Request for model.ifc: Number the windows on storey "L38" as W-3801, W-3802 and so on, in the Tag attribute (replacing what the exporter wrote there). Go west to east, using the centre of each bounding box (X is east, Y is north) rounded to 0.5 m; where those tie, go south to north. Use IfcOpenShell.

First a look at what the model holds.

```python
import ifcopenshell
import ifcopenshell.util.element
import ifcopenshell.util.placement

model = ifcopenshell.open("model.ifc")
print(model.schema)
storey = next(s for s in model.by_type("IfcBuildingStorey") if s.Name == "L38")
windows = [e for e in ifcopenshell.util.element.get_decomposition(storey) if e.is_a("IfcWindow")]
for e in sorted(windows, key=lambda e: e.id()):
    origin = ifcopenshell.util.placement.get_local_placement(e.ObjectPlacement)[:3, 3]
    print(e.id(), e.Tag, e.Name, origin.round(2) + 0.0, sep=" | ")
```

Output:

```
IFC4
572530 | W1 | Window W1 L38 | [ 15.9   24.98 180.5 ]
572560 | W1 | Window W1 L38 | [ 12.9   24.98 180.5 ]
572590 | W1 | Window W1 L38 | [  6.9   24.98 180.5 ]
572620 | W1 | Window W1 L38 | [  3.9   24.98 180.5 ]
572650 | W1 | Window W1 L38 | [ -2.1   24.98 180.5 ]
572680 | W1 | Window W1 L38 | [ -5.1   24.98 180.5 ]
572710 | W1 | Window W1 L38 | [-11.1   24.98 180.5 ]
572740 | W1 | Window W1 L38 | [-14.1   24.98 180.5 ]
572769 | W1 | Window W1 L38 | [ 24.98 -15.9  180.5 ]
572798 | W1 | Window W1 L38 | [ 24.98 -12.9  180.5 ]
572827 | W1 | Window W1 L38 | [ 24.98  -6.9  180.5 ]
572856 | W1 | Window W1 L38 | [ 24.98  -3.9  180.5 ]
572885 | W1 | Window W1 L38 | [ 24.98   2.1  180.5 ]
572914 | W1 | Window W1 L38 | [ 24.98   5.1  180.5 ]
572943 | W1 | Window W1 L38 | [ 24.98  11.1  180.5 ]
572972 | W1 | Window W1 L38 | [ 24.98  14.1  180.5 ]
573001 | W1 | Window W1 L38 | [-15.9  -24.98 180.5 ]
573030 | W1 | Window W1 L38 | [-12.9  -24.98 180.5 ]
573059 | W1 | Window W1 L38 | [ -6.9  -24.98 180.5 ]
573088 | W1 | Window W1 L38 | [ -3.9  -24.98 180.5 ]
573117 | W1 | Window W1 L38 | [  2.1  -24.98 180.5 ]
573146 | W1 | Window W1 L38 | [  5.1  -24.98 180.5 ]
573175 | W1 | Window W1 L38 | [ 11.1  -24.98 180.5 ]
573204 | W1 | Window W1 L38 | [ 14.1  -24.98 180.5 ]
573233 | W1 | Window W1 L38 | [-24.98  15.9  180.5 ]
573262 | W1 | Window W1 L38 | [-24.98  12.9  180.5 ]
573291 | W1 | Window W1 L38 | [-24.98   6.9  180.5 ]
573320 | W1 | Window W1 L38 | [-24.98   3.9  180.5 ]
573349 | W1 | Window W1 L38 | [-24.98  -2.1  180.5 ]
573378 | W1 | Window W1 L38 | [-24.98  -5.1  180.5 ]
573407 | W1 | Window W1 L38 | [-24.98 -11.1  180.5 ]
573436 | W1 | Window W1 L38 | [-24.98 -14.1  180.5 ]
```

```python
import ifcopenshell
import ifcopenshell.geom
import ifcopenshell.util.element
import ifcopenshell.util.shape

model = ifcopenshell.open("model.ifc")
settings = ifcopenshell.geom.settings()
settings.set("use-world-coords", True)


def centre(element):
    shape = ifcopenshell.geom.create_shape(settings, element)
    return ifcopenshell.util.shape.get_bbox_centroid(shape.geometry)


storey = next(s for s in model.by_type("IfcBuildingStorey") if s.Name == "L38")
windows = [e for e in ifcopenshell.util.element.get_decomposition(storey) if e.is_a("IfcWindow")]

# Insertion points can sit at a corner or the storey origin, so sort by the geometry (in metres).
centres = {e: centre(e) for e in windows}
windows.sort(key=lambda e: (round(centres[e][0] / 0.5), centres[e][1]))

for i, e in enumerate(windows, start=1):
    number = f"W-38{i:02d}"
    e.Tag = number
    print(e.id(), number)

model.write("model_updated.ifc")
```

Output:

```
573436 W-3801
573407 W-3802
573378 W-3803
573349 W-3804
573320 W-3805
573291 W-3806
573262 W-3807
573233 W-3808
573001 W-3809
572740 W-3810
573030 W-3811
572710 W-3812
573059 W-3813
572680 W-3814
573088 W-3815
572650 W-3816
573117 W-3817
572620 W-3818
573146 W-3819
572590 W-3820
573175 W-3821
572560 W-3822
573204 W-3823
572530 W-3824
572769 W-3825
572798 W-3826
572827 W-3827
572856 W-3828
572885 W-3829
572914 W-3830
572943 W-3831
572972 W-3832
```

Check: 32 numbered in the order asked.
